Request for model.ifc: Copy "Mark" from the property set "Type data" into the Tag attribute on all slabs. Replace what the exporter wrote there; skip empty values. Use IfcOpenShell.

First a look at what the model holds.

```python
import ifcopenshell
import ifcopenshell.util.element

model = ifcopenshell.open("model.ifc")
print(model.schema)
slabs = model.by_type("IfcSlab")
print(len(slabs), "slabs")
for e in slabs[:8]:
    source = ifcopenshell.util.element.get_pset(e, "Type data", "Mark")
    target = e.Tag
    print(e.id(), repr(source), repr(target), sep=" | ")
```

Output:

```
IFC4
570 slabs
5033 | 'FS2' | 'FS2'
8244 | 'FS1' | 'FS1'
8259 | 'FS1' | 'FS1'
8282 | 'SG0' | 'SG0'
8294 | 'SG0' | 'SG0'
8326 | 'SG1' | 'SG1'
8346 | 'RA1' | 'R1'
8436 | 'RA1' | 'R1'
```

```python
import ifcopenshell
import ifcopenshell.util.element

model = ifcopenshell.open("model.ifc")

count = 0
for e in model.by_type("IfcSlab"):
    value = ifcopenshell.util.element.get_pset(e, "Type data", "Mark")
    current = e.Tag
    if not value or not value.strip() or current == value:
        continue
    e.Tag = value
    count += 1

print(count, "slabs updated")

model.write("model_rev.ifc")
```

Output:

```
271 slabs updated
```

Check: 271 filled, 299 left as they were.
